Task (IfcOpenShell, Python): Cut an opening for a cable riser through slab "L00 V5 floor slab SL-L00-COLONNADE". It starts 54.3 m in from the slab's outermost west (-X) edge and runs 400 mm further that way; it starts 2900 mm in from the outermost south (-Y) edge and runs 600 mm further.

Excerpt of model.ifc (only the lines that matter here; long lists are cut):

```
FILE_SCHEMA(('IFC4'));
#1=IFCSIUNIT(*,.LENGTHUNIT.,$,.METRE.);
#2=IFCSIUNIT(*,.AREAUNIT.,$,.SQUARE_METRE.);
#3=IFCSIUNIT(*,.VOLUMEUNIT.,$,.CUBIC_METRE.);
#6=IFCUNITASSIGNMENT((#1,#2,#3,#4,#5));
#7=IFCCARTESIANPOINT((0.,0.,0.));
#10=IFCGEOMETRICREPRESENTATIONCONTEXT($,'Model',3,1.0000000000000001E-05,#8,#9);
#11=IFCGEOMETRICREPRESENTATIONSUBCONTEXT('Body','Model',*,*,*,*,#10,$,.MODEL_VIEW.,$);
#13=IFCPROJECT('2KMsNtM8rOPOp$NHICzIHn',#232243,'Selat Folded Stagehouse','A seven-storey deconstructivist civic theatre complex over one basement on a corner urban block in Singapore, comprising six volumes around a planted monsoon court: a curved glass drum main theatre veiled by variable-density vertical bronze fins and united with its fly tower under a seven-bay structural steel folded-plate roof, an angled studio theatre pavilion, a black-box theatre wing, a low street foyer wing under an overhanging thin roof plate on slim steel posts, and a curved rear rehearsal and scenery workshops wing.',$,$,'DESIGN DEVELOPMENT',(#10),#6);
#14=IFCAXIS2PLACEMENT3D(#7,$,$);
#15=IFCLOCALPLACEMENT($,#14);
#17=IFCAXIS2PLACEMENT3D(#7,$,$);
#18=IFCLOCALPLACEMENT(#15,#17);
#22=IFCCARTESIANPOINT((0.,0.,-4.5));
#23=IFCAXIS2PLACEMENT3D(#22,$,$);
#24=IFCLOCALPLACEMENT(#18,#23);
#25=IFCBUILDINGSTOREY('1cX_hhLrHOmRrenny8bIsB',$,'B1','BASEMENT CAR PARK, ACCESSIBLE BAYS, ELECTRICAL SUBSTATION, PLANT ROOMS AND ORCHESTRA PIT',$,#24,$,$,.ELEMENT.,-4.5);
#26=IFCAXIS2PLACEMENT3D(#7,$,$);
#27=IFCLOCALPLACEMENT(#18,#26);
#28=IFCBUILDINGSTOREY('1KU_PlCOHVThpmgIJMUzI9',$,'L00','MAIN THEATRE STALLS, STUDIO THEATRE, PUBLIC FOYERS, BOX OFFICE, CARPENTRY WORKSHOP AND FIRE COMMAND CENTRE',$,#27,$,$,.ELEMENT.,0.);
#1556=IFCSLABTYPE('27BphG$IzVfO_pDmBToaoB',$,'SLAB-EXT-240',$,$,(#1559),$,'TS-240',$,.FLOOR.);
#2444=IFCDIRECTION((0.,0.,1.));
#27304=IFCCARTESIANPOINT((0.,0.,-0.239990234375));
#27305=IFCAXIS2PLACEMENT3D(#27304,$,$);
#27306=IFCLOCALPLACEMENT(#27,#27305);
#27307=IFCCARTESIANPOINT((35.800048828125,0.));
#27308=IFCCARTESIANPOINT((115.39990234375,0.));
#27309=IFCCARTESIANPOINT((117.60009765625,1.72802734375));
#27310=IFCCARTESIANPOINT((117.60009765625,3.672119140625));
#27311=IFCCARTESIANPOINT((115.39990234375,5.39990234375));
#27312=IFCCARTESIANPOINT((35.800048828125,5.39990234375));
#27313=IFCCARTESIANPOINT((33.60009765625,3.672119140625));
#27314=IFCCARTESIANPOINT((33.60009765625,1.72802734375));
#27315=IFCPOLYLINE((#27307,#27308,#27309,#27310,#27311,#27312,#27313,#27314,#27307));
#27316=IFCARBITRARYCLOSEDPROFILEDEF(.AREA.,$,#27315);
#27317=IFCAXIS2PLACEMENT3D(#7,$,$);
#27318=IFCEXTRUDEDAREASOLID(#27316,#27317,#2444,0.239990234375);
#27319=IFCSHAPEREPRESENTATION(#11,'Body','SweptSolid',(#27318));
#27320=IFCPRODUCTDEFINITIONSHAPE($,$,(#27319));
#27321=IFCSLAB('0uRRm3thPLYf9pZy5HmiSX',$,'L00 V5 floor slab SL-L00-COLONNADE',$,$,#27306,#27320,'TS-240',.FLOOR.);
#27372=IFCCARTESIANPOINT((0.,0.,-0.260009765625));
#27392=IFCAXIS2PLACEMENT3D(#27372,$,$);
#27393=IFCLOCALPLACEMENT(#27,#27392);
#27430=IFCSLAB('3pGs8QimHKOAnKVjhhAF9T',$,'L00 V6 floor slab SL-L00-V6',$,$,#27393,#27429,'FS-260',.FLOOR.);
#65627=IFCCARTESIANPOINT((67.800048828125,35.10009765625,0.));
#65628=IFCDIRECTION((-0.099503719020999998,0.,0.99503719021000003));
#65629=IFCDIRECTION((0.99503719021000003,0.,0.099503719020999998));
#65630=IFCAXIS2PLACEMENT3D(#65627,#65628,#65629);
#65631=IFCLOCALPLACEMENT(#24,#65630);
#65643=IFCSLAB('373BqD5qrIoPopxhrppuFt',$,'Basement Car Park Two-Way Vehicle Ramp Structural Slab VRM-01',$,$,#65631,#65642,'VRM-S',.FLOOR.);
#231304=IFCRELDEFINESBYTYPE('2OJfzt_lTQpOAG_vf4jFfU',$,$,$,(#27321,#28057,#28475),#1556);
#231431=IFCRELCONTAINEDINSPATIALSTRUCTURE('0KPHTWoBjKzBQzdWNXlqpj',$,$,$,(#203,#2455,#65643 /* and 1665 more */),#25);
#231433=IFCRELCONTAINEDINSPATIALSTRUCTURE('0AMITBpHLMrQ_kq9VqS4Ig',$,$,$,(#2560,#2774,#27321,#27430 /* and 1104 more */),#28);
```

```python
import numpy as np
import ifcopenshell
import ifcopenshell.api.feature
import ifcopenshell.api.geometry
import ifcopenshell.api.root
import ifcopenshell.geom
import ifcopenshell.util.placement
import ifcopenshell.util.representation
import ifcopenshell.util.shape
import ifcopenshell.util.unit

model = ifcopenshell.open("model.ifc")
unit_scale = ifcopenshell.util.unit.calculate_unit_scale(model)
settings = ifcopenshell.geom.settings()


def volume(element):
    """Net volume in cubic metres, openings subtracted."""
    shape = ifcopenshell.geom.create_shape(settings, element)
    return ifcopenshell.util.shape.get_volume(shape.geometry)


slab = model.by_id(27321)
before = volume(slab)

# Extent in the slab's own axes, in metres. The edges named are its -X and -Y sides.
slab_shape = ifcopenshell.geom.create_shape(settings, slab)
vertices = ifcopenshell.util.shape.get_vertices(slab_shape.geometry)
x_min, y_min, bottom = vertices.min(axis=0)
top = vertices[:, 2].max()

opening = ifcopenshell.api.root.create_entity(model, ifc_class="IfcOpeningElement", name="Cable riser opening", predefined_type="OPENING")
context = ifcopenshell.util.representation.get_context(model, "Model", "Body", "MODEL_VIEW")
width, depth = 0.4, 0.6
outline = [(0.0, 0.0), (width, 0.0), (width, depth), (0.0, depth), (0.0, 0.0)]
# Overshoot both faces by 50 mm so the cut is clean.
shape = ifcopenshell.api.geometry.add_slab_representation(
    model, context=context, depth=top - bottom + 0.1, polyline=outline
)
ifcopenshell.api.geometry.assign_representation(model, product=opening, representation=shape)

matrix = ifcopenshell.util.placement.get_local_placement(slab.ObjectPlacement)
matrix[:, 3] = matrix @ np.append(np.array([x_min + 54.3, y_min + 2.9, bottom - 0.05]) / unit_scale, 1.0)
ifcopenshell.api.geometry.edit_object_placement(model, product=opening, matrix=matrix, is_si=False)
ifcopenshell.api.feature.add_feature(model, feature=opening, element=slab)

after = volume(slab)

print(f"slab volume {before:.3f} -> {after:.3f} m3")

model.write("model_updated.ifc")
```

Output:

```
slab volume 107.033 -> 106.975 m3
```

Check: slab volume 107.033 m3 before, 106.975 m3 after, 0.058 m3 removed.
